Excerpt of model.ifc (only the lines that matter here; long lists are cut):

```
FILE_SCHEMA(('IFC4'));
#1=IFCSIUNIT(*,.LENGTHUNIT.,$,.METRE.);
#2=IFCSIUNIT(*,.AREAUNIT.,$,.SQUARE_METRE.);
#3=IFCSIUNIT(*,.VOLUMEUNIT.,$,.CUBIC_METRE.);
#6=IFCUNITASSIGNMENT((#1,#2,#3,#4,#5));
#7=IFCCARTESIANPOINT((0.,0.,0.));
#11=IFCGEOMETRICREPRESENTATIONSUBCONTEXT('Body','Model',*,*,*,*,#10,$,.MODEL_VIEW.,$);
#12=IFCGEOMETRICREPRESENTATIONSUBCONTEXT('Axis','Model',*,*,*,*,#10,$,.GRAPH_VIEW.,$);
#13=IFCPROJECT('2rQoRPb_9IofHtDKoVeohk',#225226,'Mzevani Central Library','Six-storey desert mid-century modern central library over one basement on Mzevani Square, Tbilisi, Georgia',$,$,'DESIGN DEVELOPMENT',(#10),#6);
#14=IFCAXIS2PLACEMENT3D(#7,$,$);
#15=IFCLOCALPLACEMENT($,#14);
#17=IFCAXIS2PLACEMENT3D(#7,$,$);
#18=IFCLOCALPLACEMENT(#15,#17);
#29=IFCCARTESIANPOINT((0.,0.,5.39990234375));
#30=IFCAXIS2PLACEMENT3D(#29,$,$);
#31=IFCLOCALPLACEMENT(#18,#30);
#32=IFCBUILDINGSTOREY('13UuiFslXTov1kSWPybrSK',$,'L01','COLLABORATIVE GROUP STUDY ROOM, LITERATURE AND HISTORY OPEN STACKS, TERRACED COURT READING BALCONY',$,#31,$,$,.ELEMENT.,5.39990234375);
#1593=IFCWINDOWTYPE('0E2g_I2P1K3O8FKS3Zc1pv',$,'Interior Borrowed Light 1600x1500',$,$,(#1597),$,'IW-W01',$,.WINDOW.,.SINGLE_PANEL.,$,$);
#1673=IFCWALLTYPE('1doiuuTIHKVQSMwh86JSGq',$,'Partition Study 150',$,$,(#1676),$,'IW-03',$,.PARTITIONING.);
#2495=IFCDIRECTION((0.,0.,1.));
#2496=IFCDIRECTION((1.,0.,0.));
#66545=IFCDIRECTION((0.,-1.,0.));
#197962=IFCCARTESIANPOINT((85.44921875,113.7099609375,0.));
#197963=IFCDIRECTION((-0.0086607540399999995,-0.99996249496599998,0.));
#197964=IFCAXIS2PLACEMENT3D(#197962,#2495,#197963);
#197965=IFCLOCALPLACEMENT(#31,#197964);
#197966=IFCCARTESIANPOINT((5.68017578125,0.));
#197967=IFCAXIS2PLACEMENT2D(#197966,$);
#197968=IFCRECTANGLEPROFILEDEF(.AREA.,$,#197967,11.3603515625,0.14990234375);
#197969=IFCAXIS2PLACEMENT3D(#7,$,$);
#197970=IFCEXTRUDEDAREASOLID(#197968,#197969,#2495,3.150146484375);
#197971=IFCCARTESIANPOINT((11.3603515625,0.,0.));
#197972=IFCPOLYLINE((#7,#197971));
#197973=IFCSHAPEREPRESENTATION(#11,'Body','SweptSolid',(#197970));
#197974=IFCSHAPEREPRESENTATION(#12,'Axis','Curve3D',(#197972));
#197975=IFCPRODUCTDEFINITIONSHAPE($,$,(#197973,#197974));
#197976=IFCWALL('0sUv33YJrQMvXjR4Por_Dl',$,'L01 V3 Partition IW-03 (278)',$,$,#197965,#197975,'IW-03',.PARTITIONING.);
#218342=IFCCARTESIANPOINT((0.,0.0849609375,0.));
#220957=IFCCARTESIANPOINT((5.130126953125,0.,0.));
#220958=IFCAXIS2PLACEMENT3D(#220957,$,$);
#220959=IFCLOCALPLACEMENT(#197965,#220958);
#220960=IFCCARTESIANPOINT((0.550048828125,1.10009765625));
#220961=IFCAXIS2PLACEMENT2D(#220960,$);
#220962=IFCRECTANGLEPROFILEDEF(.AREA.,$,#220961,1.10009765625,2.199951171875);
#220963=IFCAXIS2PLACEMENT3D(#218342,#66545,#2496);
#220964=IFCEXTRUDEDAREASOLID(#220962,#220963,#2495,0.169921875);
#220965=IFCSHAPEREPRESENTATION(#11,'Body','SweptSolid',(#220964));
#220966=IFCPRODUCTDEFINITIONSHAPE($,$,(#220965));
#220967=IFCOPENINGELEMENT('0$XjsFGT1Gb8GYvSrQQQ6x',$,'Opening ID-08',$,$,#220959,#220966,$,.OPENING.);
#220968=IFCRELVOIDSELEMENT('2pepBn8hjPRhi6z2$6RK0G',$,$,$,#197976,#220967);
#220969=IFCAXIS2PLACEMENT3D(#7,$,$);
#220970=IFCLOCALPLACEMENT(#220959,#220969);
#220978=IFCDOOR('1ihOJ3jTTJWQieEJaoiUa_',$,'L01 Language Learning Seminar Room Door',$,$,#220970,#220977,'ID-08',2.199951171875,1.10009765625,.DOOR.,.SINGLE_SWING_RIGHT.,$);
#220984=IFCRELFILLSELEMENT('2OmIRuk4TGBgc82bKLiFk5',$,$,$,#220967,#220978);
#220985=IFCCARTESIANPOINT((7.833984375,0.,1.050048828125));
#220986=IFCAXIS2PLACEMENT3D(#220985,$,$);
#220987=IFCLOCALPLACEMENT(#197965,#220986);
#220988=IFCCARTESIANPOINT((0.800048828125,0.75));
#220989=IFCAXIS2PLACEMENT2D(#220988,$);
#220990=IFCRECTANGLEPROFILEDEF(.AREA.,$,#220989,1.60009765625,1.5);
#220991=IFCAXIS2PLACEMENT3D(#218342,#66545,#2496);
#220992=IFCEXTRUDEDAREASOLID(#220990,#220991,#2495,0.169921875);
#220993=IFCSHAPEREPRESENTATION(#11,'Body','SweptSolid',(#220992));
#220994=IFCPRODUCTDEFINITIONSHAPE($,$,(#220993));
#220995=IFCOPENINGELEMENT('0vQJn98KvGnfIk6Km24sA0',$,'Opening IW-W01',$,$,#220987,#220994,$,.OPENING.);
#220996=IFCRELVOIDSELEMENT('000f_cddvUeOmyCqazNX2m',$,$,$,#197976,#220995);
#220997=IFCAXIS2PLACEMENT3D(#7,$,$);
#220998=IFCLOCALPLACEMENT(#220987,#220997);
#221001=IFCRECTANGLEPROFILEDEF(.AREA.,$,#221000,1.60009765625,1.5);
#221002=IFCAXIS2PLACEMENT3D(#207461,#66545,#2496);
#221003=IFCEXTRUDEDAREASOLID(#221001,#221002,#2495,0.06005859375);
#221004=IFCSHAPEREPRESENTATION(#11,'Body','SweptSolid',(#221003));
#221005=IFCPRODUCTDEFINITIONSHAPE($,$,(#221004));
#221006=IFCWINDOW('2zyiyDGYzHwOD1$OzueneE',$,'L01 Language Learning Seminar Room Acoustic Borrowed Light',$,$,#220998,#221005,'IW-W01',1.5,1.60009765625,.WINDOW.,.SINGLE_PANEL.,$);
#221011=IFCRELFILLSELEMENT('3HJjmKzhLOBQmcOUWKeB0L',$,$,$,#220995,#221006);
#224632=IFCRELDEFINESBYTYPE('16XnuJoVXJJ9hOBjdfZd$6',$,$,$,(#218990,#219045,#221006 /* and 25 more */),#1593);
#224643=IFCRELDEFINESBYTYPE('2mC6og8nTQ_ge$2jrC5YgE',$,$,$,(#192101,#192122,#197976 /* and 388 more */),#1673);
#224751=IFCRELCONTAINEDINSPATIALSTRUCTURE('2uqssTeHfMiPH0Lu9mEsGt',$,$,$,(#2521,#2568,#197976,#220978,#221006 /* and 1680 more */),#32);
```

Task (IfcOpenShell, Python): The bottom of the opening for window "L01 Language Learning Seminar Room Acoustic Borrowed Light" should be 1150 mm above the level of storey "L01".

```python
import numpy as np
import ifcopenshell
import ifcopenshell.api.geometry
import ifcopenshell.geom
import ifcopenshell.util.element
import ifcopenshell.util.placement
import ifcopenshell.util.shape
import ifcopenshell.util.unit

model = ifcopenshell.open("model.ifc")
unit_scale = ifcopenshell.util.unit.calculate_unit_scale(model)

window = model.by_guid("2zyiyDGYzHwOD1$OzueneE")
opening = window.FillsVoids[0].RelatingOpeningElement
storey = ifcopenshell.util.element.get_container(window, ifc_class="IfcBuildingStorey")
level = ifcopenshell.util.placement.get_local_placement(storey.ObjectPlacement)[2, 3]

# The opening's origin need not be at the sill, so measure its lowest point.
shape = ifcopenshell.geom.create_shape(ifcopenshell.geom.settings(), opening)
bottom = ifcopenshell.util.shape.get_shape_bottom_elevation(shape, shape.geometry) / unit_scale
dz = level + 1.15 / unit_scale - bottom

shift = np.array([0.0, 0.0, dz])
# The window is placed relative to its opening, so it follows when the opening moves.
matrix = ifcopenshell.util.placement.get_local_placement(opening.ObjectPlacement)
matrix[:3, 3] += shift
ifcopenshell.api.geometry.edit_object_placement(
    model, product=opening, matrix=matrix, is_si=False, should_transform_children=True
)

print(f"moved by {dz * unit_scale:+.3f} m")

model.write("model_edited.ifc")
```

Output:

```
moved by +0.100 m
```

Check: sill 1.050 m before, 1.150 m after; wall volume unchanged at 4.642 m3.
